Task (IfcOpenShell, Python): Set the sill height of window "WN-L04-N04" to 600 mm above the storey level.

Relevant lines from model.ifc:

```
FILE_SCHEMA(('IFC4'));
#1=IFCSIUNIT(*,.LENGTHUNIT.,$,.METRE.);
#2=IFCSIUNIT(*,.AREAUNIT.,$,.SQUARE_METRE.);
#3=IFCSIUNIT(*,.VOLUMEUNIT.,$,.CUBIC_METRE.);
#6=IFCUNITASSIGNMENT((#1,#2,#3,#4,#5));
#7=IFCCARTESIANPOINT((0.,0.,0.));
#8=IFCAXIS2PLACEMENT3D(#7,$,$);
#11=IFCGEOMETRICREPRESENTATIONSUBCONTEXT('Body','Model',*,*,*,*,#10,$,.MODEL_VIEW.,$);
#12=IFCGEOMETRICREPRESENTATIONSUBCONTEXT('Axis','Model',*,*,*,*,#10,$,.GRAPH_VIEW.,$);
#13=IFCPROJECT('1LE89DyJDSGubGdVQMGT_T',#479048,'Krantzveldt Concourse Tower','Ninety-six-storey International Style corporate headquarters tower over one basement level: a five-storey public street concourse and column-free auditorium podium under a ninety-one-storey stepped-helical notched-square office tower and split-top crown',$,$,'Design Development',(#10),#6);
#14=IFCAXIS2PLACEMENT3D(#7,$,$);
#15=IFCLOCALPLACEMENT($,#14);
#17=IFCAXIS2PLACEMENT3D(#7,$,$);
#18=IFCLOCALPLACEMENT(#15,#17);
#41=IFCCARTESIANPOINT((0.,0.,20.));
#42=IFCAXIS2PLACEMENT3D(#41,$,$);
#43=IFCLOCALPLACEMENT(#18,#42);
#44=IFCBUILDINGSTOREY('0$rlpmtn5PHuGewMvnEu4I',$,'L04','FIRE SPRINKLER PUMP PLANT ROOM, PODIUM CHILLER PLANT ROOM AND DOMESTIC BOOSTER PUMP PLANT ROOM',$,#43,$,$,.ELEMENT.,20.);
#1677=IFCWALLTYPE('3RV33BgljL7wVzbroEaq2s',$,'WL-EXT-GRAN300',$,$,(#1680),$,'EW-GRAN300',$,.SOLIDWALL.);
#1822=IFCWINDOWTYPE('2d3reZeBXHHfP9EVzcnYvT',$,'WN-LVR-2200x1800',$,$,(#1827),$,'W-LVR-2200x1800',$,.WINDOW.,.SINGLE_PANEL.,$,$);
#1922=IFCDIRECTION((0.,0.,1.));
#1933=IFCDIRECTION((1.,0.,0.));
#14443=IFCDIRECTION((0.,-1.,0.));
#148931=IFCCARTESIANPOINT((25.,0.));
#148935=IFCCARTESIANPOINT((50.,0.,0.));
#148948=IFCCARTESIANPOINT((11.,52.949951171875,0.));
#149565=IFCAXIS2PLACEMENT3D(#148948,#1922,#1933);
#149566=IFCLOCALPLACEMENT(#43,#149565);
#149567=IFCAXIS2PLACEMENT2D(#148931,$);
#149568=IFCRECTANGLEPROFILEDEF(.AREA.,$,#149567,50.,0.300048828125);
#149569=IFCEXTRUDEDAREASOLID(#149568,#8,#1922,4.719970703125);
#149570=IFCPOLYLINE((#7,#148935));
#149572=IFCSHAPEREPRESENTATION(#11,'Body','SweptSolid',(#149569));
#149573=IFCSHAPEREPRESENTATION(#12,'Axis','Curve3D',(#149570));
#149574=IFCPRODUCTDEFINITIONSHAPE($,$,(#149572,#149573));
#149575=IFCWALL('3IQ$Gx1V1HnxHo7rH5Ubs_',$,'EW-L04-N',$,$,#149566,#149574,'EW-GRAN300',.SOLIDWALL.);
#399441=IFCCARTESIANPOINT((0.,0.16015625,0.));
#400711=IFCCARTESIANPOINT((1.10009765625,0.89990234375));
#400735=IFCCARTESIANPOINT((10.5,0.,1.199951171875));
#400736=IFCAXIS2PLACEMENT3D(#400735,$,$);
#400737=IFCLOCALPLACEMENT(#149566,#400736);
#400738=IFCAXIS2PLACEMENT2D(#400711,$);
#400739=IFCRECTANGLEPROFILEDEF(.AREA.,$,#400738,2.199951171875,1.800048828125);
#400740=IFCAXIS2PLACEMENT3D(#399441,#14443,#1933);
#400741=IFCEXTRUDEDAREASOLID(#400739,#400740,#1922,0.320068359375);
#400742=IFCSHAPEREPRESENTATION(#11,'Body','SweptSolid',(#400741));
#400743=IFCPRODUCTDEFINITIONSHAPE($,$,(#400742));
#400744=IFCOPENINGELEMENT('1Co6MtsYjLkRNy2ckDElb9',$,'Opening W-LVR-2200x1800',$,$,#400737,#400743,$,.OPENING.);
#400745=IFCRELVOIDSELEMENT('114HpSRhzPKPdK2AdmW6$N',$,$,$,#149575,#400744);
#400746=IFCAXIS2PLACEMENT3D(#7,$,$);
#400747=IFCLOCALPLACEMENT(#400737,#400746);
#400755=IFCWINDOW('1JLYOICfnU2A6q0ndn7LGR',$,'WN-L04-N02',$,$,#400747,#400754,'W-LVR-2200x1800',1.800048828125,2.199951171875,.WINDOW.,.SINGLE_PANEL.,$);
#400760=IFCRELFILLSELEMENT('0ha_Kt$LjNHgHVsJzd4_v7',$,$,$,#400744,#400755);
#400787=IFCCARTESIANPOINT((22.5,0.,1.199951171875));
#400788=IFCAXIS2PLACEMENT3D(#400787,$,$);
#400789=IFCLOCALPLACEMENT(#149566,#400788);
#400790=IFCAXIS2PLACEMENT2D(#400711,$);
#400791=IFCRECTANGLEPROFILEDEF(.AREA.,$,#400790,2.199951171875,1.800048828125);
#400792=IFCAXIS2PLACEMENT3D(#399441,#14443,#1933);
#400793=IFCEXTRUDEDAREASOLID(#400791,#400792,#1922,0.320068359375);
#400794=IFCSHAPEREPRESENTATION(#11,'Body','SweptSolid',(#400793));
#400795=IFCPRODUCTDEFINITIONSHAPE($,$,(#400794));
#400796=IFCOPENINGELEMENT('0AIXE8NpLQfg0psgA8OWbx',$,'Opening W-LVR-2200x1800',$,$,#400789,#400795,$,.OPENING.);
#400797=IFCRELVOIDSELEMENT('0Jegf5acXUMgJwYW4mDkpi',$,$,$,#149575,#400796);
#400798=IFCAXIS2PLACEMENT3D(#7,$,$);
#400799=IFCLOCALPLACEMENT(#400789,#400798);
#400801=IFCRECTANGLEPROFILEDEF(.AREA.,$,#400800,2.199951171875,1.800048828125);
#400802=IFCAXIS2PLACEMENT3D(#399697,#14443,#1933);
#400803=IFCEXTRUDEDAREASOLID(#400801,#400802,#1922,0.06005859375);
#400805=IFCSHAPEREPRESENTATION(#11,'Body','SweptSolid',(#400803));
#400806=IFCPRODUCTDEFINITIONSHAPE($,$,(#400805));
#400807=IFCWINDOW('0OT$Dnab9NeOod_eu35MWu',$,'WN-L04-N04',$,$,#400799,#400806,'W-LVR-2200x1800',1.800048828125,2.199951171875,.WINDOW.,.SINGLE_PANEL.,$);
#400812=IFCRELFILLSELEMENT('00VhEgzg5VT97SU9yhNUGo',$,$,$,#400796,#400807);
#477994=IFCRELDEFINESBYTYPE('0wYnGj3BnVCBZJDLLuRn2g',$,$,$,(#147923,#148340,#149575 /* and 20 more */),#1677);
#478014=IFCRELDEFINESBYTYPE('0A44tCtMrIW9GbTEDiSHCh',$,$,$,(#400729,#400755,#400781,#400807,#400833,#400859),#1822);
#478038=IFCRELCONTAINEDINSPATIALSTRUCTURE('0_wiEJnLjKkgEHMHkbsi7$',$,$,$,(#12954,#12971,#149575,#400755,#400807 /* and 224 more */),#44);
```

```python
import numpy as np
import ifcopenshell
import ifcopenshell.api.geometry
import ifcopenshell.geom
import ifcopenshell.util.element
import ifcopenshell.util.placement
import ifcopenshell.util.shape
import ifcopenshell.util.unit

model = ifcopenshell.open("model.ifc")
unit_scale = ifcopenshell.util.unit.calculate_unit_scale(model)

window = model.by_guid("0OT$Dnab9NeOod_eu35MWu")
opening = window.FillsVoids[0].RelatingOpeningElement
storey = ifcopenshell.util.element.get_container(window, ifc_class="IfcBuildingStorey")
level = ifcopenshell.util.placement.get_local_placement(storey.ObjectPlacement)[2, 3]

# The opening's origin need not be at the sill, so measure its lowest point.
shape = ifcopenshell.geom.create_shape(ifcopenshell.geom.settings(), opening)
bottom = ifcopenshell.util.shape.get_shape_bottom_elevation(shape, shape.geometry) / unit_scale
dz = level + 0.6 / unit_scale - bottom

shift = np.array([0.0, 0.0, dz])
# The window is placed relative to its opening, so it follows when the opening moves.
matrix = ifcopenshell.util.placement.get_local_placement(opening.ObjectPlacement)
matrix[:3, 3] += shift
ifcopenshell.api.geometry.edit_object_placement(
    model, product=opening, matrix=matrix, is_si=False, should_transform_children=True
)

print(f"moved by {dz * unit_scale:+.3f} m")

model.write("model-out.ifc")
```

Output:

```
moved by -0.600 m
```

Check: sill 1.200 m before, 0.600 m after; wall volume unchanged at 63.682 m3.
